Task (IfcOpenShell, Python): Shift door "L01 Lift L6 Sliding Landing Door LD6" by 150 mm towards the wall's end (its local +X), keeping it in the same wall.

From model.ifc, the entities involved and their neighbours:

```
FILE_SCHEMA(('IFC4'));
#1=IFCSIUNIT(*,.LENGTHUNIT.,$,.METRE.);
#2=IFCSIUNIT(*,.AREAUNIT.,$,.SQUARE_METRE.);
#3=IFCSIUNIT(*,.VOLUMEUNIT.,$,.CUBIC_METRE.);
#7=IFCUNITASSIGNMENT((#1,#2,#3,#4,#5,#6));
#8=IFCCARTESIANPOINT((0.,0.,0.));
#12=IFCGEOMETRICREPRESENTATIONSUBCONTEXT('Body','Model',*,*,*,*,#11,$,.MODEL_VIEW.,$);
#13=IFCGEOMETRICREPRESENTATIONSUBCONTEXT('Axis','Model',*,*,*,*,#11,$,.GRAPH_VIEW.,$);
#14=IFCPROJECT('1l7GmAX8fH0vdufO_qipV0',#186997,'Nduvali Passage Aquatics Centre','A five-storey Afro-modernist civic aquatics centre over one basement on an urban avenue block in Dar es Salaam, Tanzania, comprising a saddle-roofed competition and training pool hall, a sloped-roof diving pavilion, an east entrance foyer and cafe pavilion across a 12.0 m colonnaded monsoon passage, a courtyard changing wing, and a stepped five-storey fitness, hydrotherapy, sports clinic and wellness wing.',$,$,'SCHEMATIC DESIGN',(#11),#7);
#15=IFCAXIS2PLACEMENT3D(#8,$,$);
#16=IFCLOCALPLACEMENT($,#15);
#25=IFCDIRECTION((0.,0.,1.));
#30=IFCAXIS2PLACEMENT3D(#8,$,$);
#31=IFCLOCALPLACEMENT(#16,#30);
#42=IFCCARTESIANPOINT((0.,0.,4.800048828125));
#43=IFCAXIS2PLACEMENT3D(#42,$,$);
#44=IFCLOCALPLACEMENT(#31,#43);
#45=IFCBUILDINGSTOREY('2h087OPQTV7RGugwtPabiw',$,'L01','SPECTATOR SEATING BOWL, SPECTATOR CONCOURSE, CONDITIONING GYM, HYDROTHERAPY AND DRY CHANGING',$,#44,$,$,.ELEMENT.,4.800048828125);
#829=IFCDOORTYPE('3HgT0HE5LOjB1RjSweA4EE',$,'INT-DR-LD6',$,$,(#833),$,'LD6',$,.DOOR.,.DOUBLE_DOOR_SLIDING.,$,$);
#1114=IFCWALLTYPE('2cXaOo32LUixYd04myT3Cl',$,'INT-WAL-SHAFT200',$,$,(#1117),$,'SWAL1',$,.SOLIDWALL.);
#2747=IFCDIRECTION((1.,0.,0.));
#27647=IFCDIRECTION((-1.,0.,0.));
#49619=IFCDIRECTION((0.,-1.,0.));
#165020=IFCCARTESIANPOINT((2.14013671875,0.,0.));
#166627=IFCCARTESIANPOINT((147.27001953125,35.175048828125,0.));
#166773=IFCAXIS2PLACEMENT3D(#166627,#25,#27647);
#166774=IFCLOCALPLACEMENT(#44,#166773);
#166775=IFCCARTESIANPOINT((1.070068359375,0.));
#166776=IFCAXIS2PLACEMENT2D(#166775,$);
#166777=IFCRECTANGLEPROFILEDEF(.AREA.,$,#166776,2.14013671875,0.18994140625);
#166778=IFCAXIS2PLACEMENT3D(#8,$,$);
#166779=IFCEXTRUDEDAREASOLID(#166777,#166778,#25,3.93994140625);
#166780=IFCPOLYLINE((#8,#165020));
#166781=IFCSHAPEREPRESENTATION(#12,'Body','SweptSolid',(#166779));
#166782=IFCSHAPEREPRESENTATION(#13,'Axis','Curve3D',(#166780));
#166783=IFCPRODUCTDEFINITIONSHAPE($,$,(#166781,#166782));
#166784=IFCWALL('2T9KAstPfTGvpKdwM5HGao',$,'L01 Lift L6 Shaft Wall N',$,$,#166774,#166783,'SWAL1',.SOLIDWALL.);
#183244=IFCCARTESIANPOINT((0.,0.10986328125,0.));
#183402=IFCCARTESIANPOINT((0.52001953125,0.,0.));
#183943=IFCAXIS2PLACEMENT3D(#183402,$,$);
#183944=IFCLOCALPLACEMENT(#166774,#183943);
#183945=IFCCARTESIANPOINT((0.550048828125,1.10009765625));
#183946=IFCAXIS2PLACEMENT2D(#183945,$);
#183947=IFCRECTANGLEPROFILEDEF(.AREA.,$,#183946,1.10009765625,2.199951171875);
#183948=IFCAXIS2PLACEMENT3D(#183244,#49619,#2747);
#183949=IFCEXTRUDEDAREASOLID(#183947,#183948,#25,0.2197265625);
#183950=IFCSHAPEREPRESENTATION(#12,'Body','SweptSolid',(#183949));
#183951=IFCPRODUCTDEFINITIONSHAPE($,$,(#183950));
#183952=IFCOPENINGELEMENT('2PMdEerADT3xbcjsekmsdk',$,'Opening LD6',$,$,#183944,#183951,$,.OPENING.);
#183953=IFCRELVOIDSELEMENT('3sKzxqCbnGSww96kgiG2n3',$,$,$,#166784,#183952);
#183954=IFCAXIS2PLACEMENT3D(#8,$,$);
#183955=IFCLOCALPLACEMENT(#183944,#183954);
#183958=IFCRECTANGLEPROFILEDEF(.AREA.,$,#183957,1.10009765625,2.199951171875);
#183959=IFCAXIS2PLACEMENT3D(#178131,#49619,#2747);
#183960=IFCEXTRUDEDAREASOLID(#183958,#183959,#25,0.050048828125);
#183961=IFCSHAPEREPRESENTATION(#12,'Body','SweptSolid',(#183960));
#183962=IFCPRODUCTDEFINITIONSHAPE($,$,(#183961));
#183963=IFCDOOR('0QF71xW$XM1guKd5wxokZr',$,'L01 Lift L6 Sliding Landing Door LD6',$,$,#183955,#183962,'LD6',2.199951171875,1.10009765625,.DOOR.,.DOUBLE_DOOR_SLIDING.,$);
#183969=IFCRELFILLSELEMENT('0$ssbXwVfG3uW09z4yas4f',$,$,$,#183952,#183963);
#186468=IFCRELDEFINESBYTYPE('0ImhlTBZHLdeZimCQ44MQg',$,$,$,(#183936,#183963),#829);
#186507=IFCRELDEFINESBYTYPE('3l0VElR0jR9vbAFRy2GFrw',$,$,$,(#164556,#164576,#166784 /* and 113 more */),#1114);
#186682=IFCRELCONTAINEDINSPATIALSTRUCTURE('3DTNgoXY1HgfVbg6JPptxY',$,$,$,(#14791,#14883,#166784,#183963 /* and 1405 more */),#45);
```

```python
import ifcopenshell
import ifcopenshell.api.geometry
import ifcopenshell.util.placement
import ifcopenshell.util.unit

model = ifcopenshell.open("model.ifc")
unit_scale = ifcopenshell.util.unit.calculate_unit_scale(model)

door = model.by_guid("0QF71xW$XM1guKd5wxokZr")
opening = door.FillsVoids[0].RelatingOpeningElement
wall = opening.VoidsElements[0].RelatingBuildingElement

wall_matrix = ifcopenshell.util.placement.get_local_placement(wall.ObjectPlacement)
shift = wall_matrix[:3, 0] * 0.15 / unit_scale
before = ifcopenshell.util.placement.get_local_placement(door.ObjectPlacement)[:3, 3].copy()

# The door is placed relative to its opening, so it follows when the opening moves.
matrix = ifcopenshell.util.placement.get_local_placement(opening.ObjectPlacement)
matrix[:3, 3] += shift
ifcopenshell.api.geometry.edit_object_placement(
    model, product=opening, matrix=matrix, is_si=False, should_transform_children=True
)

after = ifcopenshell.util.placement.get_local_placement(door.ObjectPlacement)[:3, 3]
print("door moved by", (after - before).round(3) + 0.0)

model.write("model-out.ifc")
```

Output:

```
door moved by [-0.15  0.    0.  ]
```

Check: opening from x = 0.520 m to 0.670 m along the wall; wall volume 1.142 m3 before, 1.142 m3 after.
